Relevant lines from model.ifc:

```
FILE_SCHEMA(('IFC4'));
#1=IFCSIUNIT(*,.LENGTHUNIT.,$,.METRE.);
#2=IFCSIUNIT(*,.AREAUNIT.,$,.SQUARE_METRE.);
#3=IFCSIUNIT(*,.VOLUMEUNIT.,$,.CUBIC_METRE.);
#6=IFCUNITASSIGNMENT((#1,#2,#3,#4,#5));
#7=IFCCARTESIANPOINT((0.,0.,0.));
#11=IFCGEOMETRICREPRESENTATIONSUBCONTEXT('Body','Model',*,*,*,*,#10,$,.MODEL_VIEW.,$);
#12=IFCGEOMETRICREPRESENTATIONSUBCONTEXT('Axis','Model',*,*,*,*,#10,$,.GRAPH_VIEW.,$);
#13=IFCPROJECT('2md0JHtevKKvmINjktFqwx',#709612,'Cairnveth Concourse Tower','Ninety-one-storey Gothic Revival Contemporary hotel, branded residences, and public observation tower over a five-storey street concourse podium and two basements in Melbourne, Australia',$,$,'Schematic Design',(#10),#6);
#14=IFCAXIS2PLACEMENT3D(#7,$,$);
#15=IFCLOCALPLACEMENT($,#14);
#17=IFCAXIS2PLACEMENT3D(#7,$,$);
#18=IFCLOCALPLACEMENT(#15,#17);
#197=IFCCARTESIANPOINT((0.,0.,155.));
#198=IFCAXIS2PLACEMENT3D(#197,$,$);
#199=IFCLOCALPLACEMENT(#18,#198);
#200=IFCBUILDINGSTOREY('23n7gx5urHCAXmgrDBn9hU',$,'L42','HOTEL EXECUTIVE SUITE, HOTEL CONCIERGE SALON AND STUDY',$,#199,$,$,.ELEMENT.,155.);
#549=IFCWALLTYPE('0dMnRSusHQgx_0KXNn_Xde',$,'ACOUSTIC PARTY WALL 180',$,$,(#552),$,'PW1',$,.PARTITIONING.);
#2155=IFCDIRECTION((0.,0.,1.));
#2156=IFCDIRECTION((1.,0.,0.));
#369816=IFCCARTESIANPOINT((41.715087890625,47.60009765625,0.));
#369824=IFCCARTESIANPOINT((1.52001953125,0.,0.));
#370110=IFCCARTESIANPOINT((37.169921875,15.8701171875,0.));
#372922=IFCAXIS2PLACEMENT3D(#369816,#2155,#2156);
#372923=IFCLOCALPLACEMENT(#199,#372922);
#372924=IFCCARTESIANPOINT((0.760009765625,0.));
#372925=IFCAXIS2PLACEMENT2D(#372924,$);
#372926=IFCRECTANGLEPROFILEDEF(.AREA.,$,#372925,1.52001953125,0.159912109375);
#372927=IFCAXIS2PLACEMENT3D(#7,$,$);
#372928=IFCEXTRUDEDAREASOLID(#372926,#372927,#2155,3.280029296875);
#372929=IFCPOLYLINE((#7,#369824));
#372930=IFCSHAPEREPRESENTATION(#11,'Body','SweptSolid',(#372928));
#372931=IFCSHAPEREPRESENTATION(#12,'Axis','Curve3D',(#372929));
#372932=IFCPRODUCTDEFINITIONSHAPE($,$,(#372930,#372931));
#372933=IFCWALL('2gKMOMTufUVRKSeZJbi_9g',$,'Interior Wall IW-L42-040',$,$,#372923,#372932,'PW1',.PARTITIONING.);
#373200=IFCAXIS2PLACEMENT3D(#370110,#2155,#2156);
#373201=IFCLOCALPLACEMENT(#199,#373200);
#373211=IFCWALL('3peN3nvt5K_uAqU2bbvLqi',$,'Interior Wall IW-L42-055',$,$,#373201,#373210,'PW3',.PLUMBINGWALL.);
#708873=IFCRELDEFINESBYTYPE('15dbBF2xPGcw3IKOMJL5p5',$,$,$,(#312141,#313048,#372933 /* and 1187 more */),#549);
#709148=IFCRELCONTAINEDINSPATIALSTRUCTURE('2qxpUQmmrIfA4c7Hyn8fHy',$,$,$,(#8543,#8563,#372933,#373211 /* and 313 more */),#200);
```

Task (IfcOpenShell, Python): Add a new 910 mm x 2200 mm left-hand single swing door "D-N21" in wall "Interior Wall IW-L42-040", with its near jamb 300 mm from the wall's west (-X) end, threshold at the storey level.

```python
import numpy as np
import ifcopenshell
import ifcopenshell.api.feature
import ifcopenshell.api.geometry
import ifcopenshell.api.root
import ifcopenshell.api.spatial
import ifcopenshell.geom
import ifcopenshell.util.element
import ifcopenshell.util.placement
import ifcopenshell.util.representation
import ifcopenshell.util.shape
import ifcopenshell.util.unit

model = ifcopenshell.open("model.ifc")
unit_scale = ifcopenshell.util.unit.calculate_unit_scale(model)
settings = ifcopenshell.geom.settings()


def volume(element):
    """Net volume in cubic metres, openings subtracted."""
    shape = ifcopenshell.geom.create_shape(settings, element)
    return ifcopenshell.util.shape.get_volume(shape.geometry)


wall = model.by_guid("2gKMOMTufUVRKSeZJbi_9g")
storey = ifcopenshell.util.element.get_container(wall, ifc_class="IfcBuildingStorey")
context = ifcopenshell.util.representation.get_context(model, "Model", "Body", "MODEL_VIEW")
before = volume(wall)

width, height, from_end, sill = 0.91, 2.2, 0.3, 0.0  # metres

# The wall runs along its own X axis, and the end named is its -X end.
wall_shape = ifcopenshell.geom.create_shape(settings, wall)
x, y, z = ifcopenshell.util.shape.get_vertices(wall_shape.geometry).T
start = x.min() + from_end
face, thickness = float(y.min()), float(y.max() - y.min())
wall_matrix = ifcopenshell.util.placement.get_local_placement(wall.ObjectPlacement)
level = ifcopenshell.util.placement.get_local_placement(storey.ObjectPlacement)[2, 3]


def in_wall(x, y):
    """Placement at x, y metres in the wall's axes, at sill height."""
    matrix = wall_matrix.copy()
    matrix[:, 3] = wall_matrix @ np.array([x / unit_scale, y / unit_scale, 0.0, 1.0])
    matrix[2, 3] = level + sill / unit_scale
    return matrix


# Opening: a box that overshoots both wall faces by 50 mm.
opening = ifcopenshell.api.root.create_entity(model, ifc_class="IfcOpeningElement", predefined_type="OPENING")
box = ifcopenshell.api.geometry.add_wall_representation(
    model, context=context, length=width, height=height, thickness=thickness + 0.1
)
ifcopenshell.api.geometry.assign_representation(model, product=opening, representation=box)
ifcopenshell.api.geometry.edit_object_placement(model, product=opening, matrix=in_wall(start, face - 0.05), is_si=False)
ifcopenshell.api.feature.add_feature(model, feature=opening, element=wall)

door = ifcopenshell.api.root.create_entity(model, ifc_class="IfcDoor", name="D-N21", predefined_type="DOOR")
door.OverallWidth, door.OverallHeight = width / unit_scale, height / unit_scale
door.OperationType = "SINGLE_SWING_LEFT"
body = ifcopenshell.api.geometry.add_door_representation(
    model,
    context=context,
    overall_width=door.OverallWidth,
    overall_height=door.OverallHeight,
    operation_type="SINGLE_SWING_LEFT",
    lining_properties={"LiningDepth": thickness / unit_scale, "ThresholdDepth": thickness / unit_scale},
)
ifcopenshell.api.geometry.assign_representation(model, product=door, representation=body)
ifcopenshell.api.spatial.assign_container(model, products=[door], relating_structure=storey)
ifcopenshell.api.feature.add_filling(model, opening=opening, element=door)

# The lining spans the wall, so the door starts at the wall face.
ifcopenshell.api.geometry.edit_object_placement(model, product=door, matrix=in_wall(start, face), is_si=False)

after = volume(wall)

print(f"wall volume {before:.3f} -> {after:.3f} m3")

model.write("model_v2.ifc")
```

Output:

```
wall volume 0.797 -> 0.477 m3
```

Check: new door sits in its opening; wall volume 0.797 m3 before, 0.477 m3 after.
